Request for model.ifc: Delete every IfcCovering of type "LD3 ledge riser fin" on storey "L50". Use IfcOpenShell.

First a look at what the model holds.

```python
import ifcopenshell
import ifcopenshell.util.element

model = ifcopenshell.open("model.ifc")
print(model.schema)
storey = next(s for s in model.by_type("IfcBuildingStorey") if s.Name == "L50")
coverings = [e for e in ifcopenshell.util.element.get_decomposition(storey) if e.is_a("IfcCovering")]
seen = {}
for e in coverings:
    element_type = ifcopenshell.util.element.get_type(e)
    name = element_type.Name if element_type not in (None, e) else None
    seen[name] = seen.get(name, 0) + 1
for name, count in sorted(seen.items(), key=str):
    print(count, "x", name)
```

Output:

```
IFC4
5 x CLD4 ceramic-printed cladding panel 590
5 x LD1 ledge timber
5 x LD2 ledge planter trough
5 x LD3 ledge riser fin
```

```python
import ifcopenshell
import ifcopenshell.api.root
import ifcopenshell.util.element

model = ifcopenshell.open("model.ifc")

storey = next(s for s in model.by_type("IfcBuildingStorey") if s.Name == "L50")
coverings = [e for e in ifcopenshell.util.element.get_decomposition(storey) if e.is_a("IfcCovering")]
targets = [e for e in coverings if (t := ifcopenshell.util.element.get_type(e)) not in (None, e) and t.Name == "LD3 ledge riser fin"]

for e in targets:
    ifcopenshell.api.root.remove_product(model, product=e)
print(len(targets), "removed")

model.write("model_updated.ifc")
```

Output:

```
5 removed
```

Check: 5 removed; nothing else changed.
